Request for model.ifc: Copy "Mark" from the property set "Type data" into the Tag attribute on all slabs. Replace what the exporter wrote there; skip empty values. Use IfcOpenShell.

First a look at what the model holds.

```python
import ifcopenshell
import ifcopenshell.util.element

model = ifcopenshell.open("model.ifc")
print(model.schema)
slabs = model.by_type("IfcSlab")
print(len(slabs), "slabs")
for e in slabs[:8]:
    source = ifcopenshell.util.element.get_pset(e, "Type data", "Mark")
    target = e.Tag
    print(e.id(), repr(source), repr(target), sep=" | ")
```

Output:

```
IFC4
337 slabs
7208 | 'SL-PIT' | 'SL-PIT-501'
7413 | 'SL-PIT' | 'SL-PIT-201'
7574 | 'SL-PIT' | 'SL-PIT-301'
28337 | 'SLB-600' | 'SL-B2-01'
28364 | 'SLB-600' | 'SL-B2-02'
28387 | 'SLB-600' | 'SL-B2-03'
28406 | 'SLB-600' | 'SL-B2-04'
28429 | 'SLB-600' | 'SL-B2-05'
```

```python
import ifcopenshell
import ifcopenshell.util.element

model = ifcopenshell.open("model.ifc")

count = 0
for e in model.by_type("IfcSlab"):
    value = ifcopenshell.util.element.get_pset(e, "Type data", "Mark")
    current = e.Tag
    if not value or not value.strip() or current == value:
        continue
    e.Tag = value
    count += 1

print(count, "slabs updated")

model.write("model_edited.ifc")
```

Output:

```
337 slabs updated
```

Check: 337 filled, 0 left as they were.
